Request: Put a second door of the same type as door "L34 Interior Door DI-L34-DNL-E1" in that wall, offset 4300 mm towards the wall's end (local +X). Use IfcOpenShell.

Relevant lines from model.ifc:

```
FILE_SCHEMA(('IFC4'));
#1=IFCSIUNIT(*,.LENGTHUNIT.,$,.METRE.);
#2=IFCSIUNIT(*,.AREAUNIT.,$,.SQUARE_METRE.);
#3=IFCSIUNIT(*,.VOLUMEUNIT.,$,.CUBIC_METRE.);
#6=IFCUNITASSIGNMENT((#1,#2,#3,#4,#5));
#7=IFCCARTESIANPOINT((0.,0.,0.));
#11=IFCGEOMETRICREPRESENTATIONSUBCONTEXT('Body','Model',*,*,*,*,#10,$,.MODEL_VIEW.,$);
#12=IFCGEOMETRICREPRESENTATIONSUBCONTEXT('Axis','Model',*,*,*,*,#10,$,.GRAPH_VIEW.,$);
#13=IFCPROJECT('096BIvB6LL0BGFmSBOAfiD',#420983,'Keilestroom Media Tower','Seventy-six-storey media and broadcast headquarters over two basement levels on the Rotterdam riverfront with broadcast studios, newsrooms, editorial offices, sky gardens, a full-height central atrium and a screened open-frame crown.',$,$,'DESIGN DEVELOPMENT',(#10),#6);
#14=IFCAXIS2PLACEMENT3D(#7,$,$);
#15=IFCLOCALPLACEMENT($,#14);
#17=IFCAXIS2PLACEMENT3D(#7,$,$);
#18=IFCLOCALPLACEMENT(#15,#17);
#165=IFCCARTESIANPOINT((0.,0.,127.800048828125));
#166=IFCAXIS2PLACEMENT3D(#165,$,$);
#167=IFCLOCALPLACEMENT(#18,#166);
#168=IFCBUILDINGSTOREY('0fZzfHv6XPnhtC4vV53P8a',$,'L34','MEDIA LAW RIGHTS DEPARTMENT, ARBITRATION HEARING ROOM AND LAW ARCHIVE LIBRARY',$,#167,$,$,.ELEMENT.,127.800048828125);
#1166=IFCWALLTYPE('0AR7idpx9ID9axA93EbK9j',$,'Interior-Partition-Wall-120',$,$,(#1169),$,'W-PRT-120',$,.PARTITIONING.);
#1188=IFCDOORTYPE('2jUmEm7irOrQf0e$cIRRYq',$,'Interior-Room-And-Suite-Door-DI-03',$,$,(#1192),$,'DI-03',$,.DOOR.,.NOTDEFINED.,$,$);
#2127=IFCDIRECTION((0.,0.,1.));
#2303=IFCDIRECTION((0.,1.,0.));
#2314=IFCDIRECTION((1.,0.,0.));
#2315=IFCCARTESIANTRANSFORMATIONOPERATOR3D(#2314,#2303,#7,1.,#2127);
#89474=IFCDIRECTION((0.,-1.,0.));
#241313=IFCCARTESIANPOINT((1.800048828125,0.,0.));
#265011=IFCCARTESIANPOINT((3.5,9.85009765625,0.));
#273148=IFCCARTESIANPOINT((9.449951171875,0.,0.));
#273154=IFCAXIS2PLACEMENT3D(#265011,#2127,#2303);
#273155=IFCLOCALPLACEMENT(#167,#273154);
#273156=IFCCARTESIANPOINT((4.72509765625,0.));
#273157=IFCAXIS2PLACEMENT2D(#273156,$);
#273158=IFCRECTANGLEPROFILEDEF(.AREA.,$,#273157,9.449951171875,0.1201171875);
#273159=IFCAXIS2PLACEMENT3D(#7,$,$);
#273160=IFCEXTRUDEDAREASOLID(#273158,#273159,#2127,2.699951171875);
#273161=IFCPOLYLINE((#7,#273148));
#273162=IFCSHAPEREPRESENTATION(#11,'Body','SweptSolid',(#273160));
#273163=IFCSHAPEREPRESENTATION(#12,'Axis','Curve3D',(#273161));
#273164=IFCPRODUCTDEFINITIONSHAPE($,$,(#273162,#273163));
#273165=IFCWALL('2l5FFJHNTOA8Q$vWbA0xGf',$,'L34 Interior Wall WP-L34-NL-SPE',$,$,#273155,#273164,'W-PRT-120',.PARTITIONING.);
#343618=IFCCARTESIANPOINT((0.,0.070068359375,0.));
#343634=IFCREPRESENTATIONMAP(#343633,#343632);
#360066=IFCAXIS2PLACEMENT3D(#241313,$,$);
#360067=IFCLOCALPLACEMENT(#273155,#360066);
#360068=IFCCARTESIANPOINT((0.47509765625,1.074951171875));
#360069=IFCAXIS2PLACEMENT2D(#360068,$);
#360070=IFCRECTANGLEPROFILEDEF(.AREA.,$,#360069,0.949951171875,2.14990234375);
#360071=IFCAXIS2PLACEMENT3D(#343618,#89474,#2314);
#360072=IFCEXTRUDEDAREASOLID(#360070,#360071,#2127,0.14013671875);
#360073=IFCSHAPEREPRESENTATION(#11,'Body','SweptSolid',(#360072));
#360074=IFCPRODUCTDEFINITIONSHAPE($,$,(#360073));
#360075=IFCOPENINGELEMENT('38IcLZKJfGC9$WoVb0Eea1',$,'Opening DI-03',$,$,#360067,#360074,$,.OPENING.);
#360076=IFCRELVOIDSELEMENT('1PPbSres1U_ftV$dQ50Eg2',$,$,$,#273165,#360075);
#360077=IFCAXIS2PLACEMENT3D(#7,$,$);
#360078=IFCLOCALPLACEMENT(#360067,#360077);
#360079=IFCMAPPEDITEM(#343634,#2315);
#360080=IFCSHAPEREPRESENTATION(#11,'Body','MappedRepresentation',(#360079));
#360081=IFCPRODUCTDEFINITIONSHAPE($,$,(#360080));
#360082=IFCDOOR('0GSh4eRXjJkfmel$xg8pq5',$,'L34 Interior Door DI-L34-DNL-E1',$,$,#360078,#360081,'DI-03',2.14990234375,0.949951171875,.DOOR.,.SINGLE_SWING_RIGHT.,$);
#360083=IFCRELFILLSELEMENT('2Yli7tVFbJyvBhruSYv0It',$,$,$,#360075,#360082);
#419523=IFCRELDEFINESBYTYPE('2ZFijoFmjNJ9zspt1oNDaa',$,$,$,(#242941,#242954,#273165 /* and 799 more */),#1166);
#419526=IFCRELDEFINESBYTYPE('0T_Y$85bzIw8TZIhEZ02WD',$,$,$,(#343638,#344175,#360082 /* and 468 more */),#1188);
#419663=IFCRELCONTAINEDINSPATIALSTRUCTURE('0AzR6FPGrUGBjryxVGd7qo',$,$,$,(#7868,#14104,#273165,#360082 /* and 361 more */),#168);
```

```python
import ifcopenshell
import ifcopenshell.api.feature
import ifcopenshell.api.geometry
import ifcopenshell.api.root
import ifcopenshell.geom
import ifcopenshell.util.element
import ifcopenshell.util.placement
import ifcopenshell.util.shape

model = ifcopenshell.open("model.ifc")
settings = ifcopenshell.geom.settings()


def volume(element):
    """Net volume in cubic metres, openings subtracted."""
    shape = ifcopenshell.geom.create_shape(settings, element)
    return ifcopenshell.util.shape.get_volume(shape.geometry)


door = model.by_guid("0GSh4eRXjJkfmel$xg8pq5")
opening = door.FillsVoids[0].RelatingOpeningElement
wall = opening.VoidsElements[0].RelatingBuildingElement
before = volume(wall)
shift = ifcopenshell.util.placement.get_local_placement(wall.ObjectPlacement)[:3, 0] * 4.3

# copy_class copies the void relationship, type, container and properties, but no geometry.
new_opening = ifcopenshell.api.root.copy_class(model, product=opening)
new_opening.Representation = ifcopenshell.util.element.copy_deep(
    model, opening.Representation, exclude=["IfcGeometricRepresentationContext", "IfcRepresentationMap"]
)
new_door = ifcopenshell.api.root.copy_class(model, product=door)
new_door.Representation = ifcopenshell.util.element.copy_deep(
    model, door.Representation, exclude=["IfcGeometricRepresentationContext", "IfcRepresentationMap"]
)
new_door.Tag = None
ifcopenshell.api.feature.add_filling(model, opening=new_opening, element=new_door)

for old, new in ((opening, new_opening), (door, new_door)):
    matrix = ifcopenshell.util.placement.get_local_placement(old.ObjectPlacement)
    matrix[:3, 3] += shift
    ifcopenshell.api.geometry.edit_object_placement(model, product=new, matrix=matrix, is_si=False)

after = volume(wall)

print(f"wall volume {before:.3f} -> {after:.3f} m3")

model.write("model_updated.ifc")
```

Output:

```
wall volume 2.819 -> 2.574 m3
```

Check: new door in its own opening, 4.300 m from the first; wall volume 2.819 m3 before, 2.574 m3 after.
